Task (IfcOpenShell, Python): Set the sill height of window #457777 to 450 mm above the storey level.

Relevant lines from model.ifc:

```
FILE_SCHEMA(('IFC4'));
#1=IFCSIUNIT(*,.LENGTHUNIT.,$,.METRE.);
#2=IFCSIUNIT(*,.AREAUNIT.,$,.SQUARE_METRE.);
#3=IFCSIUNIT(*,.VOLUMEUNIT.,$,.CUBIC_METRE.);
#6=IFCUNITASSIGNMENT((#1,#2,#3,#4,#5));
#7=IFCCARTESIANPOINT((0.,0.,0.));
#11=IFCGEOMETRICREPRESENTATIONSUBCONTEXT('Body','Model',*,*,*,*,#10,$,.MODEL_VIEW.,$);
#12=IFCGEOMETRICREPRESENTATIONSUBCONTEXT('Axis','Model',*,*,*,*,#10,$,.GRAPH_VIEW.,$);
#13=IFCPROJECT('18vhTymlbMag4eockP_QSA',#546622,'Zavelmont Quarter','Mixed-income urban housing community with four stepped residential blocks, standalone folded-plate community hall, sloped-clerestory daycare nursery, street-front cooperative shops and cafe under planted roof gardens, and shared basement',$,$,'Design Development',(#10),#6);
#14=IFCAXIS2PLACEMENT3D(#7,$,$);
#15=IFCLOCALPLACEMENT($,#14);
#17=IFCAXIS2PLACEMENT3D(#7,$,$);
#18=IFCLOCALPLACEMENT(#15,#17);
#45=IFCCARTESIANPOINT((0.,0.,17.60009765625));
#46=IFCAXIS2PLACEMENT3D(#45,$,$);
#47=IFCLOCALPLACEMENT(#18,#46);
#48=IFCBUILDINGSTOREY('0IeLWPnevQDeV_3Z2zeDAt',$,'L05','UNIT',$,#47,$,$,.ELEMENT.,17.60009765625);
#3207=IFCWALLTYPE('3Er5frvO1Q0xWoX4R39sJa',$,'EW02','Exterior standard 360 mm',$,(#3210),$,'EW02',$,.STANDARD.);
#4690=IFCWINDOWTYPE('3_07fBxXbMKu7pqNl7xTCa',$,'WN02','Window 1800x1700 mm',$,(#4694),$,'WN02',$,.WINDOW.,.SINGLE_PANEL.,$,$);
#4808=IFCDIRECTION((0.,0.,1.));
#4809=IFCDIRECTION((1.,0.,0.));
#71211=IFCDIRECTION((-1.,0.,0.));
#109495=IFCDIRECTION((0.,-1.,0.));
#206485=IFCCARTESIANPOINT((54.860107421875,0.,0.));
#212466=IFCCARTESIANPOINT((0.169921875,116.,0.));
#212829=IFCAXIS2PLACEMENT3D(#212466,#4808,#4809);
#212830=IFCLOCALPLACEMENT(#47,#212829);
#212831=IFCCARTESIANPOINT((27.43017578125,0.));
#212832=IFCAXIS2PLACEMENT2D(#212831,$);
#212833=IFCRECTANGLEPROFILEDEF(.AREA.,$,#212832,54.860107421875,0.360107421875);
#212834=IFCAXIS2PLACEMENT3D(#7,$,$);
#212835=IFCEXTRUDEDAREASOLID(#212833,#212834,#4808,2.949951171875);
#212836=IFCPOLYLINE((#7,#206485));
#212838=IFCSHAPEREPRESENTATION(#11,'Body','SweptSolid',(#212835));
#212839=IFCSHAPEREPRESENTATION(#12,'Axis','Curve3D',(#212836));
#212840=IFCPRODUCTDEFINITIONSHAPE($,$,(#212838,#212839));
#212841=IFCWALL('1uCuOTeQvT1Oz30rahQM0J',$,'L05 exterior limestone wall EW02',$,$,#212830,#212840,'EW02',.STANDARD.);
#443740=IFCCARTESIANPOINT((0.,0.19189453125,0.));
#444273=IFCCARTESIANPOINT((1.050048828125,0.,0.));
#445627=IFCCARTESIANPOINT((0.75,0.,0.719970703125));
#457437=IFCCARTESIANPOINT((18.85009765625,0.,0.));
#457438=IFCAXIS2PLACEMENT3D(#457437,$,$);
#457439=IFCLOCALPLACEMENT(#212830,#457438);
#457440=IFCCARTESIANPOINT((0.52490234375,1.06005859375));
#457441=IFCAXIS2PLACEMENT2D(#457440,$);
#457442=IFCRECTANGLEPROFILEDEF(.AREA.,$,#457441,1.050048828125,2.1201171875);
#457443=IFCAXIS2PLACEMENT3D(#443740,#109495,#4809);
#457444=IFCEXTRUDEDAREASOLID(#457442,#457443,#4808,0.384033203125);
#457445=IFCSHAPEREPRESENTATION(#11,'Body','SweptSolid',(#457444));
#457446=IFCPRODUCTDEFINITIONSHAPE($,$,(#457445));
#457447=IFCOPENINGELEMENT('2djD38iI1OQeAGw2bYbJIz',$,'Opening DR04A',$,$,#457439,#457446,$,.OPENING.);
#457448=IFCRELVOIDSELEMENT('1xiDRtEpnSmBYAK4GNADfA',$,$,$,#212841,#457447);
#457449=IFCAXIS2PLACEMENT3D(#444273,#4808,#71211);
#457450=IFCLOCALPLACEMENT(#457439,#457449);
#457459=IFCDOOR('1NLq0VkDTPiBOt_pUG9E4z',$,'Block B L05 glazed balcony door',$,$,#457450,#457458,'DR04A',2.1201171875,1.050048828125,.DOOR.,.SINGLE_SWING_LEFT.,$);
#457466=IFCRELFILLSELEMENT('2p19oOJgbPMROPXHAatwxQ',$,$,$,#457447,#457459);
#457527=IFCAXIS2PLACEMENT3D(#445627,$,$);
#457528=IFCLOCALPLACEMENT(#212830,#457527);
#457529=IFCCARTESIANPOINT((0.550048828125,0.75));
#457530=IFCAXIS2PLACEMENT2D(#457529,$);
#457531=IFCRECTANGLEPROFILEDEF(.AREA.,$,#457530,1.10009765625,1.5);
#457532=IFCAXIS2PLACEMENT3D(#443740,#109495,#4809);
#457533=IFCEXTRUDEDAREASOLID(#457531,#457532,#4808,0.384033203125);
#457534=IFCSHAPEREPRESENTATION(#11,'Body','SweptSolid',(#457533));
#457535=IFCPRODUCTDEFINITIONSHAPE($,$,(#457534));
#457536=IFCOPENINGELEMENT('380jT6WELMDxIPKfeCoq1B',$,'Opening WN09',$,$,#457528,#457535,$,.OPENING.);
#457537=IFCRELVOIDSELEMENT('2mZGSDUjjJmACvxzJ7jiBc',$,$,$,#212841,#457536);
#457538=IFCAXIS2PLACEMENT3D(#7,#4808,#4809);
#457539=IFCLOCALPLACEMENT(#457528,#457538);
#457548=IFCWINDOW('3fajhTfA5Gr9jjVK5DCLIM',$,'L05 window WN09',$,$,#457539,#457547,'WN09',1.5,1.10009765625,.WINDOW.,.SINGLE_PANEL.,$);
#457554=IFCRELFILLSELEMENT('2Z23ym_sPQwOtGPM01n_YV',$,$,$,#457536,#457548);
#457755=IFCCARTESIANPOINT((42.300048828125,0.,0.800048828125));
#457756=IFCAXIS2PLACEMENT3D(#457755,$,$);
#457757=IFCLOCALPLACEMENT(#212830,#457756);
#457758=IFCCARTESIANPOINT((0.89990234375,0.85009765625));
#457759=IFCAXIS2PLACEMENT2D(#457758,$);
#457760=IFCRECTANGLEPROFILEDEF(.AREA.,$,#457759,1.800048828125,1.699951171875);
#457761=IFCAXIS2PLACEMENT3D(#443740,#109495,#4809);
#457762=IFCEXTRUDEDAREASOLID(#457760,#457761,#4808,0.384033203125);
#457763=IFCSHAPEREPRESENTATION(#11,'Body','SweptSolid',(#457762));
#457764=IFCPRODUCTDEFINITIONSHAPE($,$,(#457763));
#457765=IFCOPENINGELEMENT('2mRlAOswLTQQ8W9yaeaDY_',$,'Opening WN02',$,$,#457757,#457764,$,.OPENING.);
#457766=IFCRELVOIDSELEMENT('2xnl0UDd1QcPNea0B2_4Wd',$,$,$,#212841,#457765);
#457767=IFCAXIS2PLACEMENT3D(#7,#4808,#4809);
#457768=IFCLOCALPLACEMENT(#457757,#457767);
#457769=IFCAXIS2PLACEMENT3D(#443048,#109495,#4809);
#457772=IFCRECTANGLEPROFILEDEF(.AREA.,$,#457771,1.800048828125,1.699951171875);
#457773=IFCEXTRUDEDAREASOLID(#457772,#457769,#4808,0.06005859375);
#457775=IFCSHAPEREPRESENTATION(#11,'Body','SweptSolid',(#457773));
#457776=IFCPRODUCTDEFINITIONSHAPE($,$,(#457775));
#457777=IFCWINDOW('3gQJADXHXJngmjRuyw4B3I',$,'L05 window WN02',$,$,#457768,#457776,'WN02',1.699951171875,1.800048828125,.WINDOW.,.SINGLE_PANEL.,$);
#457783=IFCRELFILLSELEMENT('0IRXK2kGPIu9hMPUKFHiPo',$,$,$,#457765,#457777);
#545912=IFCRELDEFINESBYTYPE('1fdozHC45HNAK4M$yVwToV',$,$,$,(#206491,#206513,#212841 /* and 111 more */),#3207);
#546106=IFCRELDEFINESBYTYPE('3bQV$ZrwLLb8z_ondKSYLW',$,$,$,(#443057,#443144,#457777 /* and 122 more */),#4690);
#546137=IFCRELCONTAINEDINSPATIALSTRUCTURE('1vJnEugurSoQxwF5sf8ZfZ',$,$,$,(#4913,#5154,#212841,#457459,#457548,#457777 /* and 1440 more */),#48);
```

```python
import numpy as np
import ifcopenshell
import ifcopenshell.api.geometry
import ifcopenshell.geom
import ifcopenshell.util.element
import ifcopenshell.util.placement
import ifcopenshell.util.shape
import ifcopenshell.util.unit

model = ifcopenshell.open("model.ifc")
unit_scale = ifcopenshell.util.unit.calculate_unit_scale(model)

window = model.by_guid("3gQJADXHXJngmjRuyw4B3I")
opening = window.FillsVoids[0].RelatingOpeningElement
storey = ifcopenshell.util.element.get_container(window, ifc_class="IfcBuildingStorey")
level = ifcopenshell.util.placement.get_local_placement(storey.ObjectPlacement)[2, 3]

# The opening's origin need not be at the sill, so measure its lowest point.
shape = ifcopenshell.geom.create_shape(ifcopenshell.geom.settings(), opening)
bottom = ifcopenshell.util.shape.get_shape_bottom_elevation(shape, shape.geometry) / unit_scale
dz = level + 0.45 - bottom

shift = np.array([0.0, 0.0, dz])
# The window is placed relative to its opening, so it follows when the opening moves.
matrix = ifcopenshell.util.placement.get_local_placement(opening.ObjectPlacement)
matrix[:3, 3] += shift
ifcopenshell.api.geometry.edit_object_placement(
    model, product=opening, matrix=matrix, is_si=False, should_transform_children=True
)

print(f"moved by {dz * unit_scale:+.3f} m")

model.write("model_edited.ifc")
```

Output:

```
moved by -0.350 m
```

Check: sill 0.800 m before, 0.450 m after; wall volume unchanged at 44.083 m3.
